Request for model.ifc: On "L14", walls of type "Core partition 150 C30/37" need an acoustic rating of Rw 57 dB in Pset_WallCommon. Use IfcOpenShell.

First a look at what the model holds.

```python
import ifcopenshell
import ifcopenshell.util.element

model = ifcopenshell.open("model.ifc")
print(model.schema)
storey = next(s for s in model.by_type("IfcBuildingStorey") if s.Name == "L14")
walls = [e for e in ifcopenshell.util.element.get_decomposition(storey) if e.is_a("IfcWall")]
seen = {}
for e in walls:
    element_type = ifcopenshell.util.element.get_type(e)
    key = (element_type.Name if element_type != e and element_type else None, ifcopenshell.util.element.get_pset(e, "Pset_WallCommon", "AcousticRating"))
    seen[key] = seen.get(key, 0) + 1
for (name, value), count in sorted(seen.items(), key=str):
    print(count, "x", name, "|", value)
```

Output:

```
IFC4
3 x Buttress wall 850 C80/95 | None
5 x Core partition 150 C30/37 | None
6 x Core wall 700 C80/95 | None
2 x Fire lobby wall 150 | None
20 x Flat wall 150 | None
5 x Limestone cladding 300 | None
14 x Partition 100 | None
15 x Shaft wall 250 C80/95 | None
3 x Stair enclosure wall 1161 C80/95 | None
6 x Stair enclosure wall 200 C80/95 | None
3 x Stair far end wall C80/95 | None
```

```python
import ifcopenshell
import ifcopenshell.api.pset
import ifcopenshell.util.element

model = ifcopenshell.open("model.ifc")

storey = next(s for s in model.by_type("IfcBuildingStorey") if s.Name == "L14")
walls = [e for e in ifcopenshell.util.element.get_decomposition(storey) if e.is_a("IfcWall")]

count = 0
for e in walls:
    element_type = ifcopenshell.util.element.get_type(e)
    if element_type in (None, e) or element_type.Name != "Core partition 150 C30/37":
        continue
    found = ifcopenshell.util.element.get_pset(e, "Pset_WallCommon", should_inherit=False)
    if found:
        pset = model.by_id(found["id"])
        if len(ifcopenshell.util.element.get_elements_by_pset(pset)) > 1:
            pset = ifcopenshell.api.pset.unshare_pset(model, products=[e], pset=pset)[0]
    else:
        pset = ifcopenshell.api.pset.add_pset(model, product=e, name="Pset_WallCommon")
    ifcopenshell.api.pset.edit_pset(model, pset=pset, properties={"AcousticRating": "Rw 57 dB"})
    count += 1

print(count, "walls updated")

model.write("model_rev.ifc")
```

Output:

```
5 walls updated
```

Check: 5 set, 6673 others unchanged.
